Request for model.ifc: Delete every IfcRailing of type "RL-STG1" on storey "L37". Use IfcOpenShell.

First a look at what the model holds.

```python
import ifcopenshell
import ifcopenshell.util.element

model = ifcopenshell.open("model.ifc")
print(model.schema)
storey = next(s for s in model.by_type("IfcBuildingStorey") if s.Name == "L37")
railings = [e for e in ifcopenshell.util.element.get_decomposition(storey) if e.is_a("IfcRailing")]
seen = {}
for e in railings:
    element_type = ifcopenshell.util.element.get_type(e)
    name = element_type.Name if element_type not in (None, e) else None
    seen[name] = seen.get(name, 0) + 1
for name, count in sorted(seen.items(), key=str):
    print(count, "x", name)
```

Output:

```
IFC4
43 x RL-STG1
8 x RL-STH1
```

```python
import ifcopenshell
import ifcopenshell.api.root
import ifcopenshell.util.element

model = ifcopenshell.open("model.ifc")

storey = next(s for s in model.by_type("IfcBuildingStorey") if s.Name == "L37")
railings = [e for e in ifcopenshell.util.element.get_decomposition(storey) if e.is_a("IfcRailing")]
targets = [e for e in railings if (t := ifcopenshell.util.element.get_type(e)) not in (None, e) and t.Name == "RL-STG1"]

for e in targets:
    ifcopenshell.api.root.remove_product(model, product=e)
print(len(targets), "removed")

model.write("model-out.ifc")
```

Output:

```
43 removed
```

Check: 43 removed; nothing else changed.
